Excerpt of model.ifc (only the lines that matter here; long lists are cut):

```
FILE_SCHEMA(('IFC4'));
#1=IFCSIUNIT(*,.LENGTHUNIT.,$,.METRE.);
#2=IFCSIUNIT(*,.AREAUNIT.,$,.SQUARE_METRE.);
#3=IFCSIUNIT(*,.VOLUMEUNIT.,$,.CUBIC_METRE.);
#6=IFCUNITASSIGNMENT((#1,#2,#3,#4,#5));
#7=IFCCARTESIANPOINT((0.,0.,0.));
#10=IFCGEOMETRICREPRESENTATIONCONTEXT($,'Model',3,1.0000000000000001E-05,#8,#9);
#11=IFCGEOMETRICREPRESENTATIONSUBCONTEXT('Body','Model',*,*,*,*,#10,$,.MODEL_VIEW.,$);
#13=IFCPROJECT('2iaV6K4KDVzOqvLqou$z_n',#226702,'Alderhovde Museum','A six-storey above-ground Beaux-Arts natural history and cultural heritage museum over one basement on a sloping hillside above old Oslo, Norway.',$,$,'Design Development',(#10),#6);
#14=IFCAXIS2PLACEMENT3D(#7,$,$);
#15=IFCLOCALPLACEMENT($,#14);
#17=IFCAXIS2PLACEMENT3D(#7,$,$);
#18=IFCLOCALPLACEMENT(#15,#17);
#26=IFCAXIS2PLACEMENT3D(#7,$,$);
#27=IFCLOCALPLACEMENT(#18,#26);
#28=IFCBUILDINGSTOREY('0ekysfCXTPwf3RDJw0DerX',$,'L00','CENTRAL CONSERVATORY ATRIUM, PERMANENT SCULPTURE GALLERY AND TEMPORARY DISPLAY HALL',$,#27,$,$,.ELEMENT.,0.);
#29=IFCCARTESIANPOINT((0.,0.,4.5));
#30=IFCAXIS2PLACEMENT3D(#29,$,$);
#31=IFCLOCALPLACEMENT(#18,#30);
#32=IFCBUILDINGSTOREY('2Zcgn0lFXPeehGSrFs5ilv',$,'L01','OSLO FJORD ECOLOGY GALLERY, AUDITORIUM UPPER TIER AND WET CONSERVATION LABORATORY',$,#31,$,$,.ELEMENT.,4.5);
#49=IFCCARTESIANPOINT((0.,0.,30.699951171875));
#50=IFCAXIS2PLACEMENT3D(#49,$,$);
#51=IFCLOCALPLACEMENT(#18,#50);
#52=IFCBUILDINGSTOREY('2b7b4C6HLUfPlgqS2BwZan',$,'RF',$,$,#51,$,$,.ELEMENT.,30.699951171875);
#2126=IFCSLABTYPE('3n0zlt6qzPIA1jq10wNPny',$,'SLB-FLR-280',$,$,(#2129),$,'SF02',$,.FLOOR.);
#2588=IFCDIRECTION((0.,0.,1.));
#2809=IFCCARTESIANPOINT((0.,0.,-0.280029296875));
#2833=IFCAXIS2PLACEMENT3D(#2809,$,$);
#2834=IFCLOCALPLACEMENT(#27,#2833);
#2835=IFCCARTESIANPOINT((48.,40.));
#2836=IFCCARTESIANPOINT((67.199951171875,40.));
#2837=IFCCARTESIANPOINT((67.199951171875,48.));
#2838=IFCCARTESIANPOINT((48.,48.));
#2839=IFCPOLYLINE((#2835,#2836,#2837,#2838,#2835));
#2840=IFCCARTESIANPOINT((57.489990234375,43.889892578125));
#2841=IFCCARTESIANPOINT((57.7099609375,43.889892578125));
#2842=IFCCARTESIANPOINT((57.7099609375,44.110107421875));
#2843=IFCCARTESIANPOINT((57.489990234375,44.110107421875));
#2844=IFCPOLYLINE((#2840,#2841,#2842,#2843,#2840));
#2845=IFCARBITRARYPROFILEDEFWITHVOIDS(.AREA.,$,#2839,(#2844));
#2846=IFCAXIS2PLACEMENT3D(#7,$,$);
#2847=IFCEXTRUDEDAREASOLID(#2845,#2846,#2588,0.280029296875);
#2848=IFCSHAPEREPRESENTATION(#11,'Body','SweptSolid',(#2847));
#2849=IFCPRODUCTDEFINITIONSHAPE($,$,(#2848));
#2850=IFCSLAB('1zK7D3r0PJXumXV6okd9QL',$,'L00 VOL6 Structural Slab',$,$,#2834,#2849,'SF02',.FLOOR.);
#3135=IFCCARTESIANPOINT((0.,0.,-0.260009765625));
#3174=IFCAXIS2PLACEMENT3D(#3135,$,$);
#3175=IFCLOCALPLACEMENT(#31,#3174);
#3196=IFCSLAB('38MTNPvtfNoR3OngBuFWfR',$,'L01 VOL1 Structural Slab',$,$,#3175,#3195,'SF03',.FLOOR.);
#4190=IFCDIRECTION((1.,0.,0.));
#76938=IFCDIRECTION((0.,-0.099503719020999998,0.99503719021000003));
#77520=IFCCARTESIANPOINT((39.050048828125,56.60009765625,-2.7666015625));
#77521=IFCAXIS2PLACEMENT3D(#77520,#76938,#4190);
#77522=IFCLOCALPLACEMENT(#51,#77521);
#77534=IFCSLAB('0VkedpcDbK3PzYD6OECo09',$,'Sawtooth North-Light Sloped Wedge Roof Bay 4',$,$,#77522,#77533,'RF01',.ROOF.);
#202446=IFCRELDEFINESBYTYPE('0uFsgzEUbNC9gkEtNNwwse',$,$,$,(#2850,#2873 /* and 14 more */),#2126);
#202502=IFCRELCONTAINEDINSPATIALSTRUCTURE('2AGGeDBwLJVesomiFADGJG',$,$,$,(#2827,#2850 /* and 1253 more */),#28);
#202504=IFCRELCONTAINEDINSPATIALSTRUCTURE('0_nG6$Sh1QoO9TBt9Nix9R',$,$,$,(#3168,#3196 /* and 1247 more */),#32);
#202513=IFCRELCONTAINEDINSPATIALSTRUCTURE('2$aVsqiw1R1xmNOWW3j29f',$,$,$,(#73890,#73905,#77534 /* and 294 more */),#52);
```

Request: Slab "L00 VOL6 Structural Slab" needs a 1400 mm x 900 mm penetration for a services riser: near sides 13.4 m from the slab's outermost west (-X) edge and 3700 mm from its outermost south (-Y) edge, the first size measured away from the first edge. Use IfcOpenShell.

```python
import numpy as np
import ifcopenshell
import ifcopenshell.api.feature
import ifcopenshell.api.geometry
import ifcopenshell.api.root
import ifcopenshell.geom
import ifcopenshell.util.placement
import ifcopenshell.util.representation
import ifcopenshell.util.shape
import ifcopenshell.util.unit

model = ifcopenshell.open("model.ifc")
unit_scale = ifcopenshell.util.unit.calculate_unit_scale(model)
settings = ifcopenshell.geom.settings()


def volume(element):
    """Net volume in cubic metres, openings subtracted."""
    shape = ifcopenshell.geom.create_shape(settings, element)
    return ifcopenshell.util.shape.get_volume(shape.geometry)


slab = model.by_guid("1zK7D3r0PJXumXV6okd9QL")
before = volume(slab)

# Extent in the slab's own axes, in metres. The edges named are its -X and -Y sides.
slab_shape = ifcopenshell.geom.create_shape(settings, slab)
vertices = ifcopenshell.util.shape.get_vertices(slab_shape.geometry)
x_min, y_min, bottom = vertices.min(axis=0)
top = vertices[:, 2].max()

opening = ifcopenshell.api.root.create_entity(model, ifc_class="IfcOpeningElement", name="Services riser opening", predefined_type="OPENING")
context = ifcopenshell.util.representation.get_context(model, "Model", "Body", "MODEL_VIEW")
width, depth = 1.4, 0.9
outline = [(0.0, 0.0), (width, 0.0), (width, depth), (0.0, depth), (0.0, 0.0)]
# Overshoot both faces by 50 mm so the cut is clean.
shape = ifcopenshell.api.geometry.add_slab_representation(
    model, context=context, depth=top - bottom + 0.1, polyline=outline
)
ifcopenshell.api.geometry.assign_representation(model, product=opening, representation=shape)

matrix = ifcopenshell.util.placement.get_local_placement(slab.ObjectPlacement)
matrix[:, 3] = matrix @ np.append(np.array([x_min + 13.4, y_min + 3.7, bottom - 0.05]) / unit_scale, 1.0)
ifcopenshell.api.geometry.edit_object_placement(model, product=opening, matrix=matrix, is_si=False)
ifcopenshell.api.feature.add_feature(model, feature=opening, element=slab)

after = volume(slab)

print(f"slab volume {before:.3f} -> {after:.3f} m3")

model.write("model_edited.ifc")
```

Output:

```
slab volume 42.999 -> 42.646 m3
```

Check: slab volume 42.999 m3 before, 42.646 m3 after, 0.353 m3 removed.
